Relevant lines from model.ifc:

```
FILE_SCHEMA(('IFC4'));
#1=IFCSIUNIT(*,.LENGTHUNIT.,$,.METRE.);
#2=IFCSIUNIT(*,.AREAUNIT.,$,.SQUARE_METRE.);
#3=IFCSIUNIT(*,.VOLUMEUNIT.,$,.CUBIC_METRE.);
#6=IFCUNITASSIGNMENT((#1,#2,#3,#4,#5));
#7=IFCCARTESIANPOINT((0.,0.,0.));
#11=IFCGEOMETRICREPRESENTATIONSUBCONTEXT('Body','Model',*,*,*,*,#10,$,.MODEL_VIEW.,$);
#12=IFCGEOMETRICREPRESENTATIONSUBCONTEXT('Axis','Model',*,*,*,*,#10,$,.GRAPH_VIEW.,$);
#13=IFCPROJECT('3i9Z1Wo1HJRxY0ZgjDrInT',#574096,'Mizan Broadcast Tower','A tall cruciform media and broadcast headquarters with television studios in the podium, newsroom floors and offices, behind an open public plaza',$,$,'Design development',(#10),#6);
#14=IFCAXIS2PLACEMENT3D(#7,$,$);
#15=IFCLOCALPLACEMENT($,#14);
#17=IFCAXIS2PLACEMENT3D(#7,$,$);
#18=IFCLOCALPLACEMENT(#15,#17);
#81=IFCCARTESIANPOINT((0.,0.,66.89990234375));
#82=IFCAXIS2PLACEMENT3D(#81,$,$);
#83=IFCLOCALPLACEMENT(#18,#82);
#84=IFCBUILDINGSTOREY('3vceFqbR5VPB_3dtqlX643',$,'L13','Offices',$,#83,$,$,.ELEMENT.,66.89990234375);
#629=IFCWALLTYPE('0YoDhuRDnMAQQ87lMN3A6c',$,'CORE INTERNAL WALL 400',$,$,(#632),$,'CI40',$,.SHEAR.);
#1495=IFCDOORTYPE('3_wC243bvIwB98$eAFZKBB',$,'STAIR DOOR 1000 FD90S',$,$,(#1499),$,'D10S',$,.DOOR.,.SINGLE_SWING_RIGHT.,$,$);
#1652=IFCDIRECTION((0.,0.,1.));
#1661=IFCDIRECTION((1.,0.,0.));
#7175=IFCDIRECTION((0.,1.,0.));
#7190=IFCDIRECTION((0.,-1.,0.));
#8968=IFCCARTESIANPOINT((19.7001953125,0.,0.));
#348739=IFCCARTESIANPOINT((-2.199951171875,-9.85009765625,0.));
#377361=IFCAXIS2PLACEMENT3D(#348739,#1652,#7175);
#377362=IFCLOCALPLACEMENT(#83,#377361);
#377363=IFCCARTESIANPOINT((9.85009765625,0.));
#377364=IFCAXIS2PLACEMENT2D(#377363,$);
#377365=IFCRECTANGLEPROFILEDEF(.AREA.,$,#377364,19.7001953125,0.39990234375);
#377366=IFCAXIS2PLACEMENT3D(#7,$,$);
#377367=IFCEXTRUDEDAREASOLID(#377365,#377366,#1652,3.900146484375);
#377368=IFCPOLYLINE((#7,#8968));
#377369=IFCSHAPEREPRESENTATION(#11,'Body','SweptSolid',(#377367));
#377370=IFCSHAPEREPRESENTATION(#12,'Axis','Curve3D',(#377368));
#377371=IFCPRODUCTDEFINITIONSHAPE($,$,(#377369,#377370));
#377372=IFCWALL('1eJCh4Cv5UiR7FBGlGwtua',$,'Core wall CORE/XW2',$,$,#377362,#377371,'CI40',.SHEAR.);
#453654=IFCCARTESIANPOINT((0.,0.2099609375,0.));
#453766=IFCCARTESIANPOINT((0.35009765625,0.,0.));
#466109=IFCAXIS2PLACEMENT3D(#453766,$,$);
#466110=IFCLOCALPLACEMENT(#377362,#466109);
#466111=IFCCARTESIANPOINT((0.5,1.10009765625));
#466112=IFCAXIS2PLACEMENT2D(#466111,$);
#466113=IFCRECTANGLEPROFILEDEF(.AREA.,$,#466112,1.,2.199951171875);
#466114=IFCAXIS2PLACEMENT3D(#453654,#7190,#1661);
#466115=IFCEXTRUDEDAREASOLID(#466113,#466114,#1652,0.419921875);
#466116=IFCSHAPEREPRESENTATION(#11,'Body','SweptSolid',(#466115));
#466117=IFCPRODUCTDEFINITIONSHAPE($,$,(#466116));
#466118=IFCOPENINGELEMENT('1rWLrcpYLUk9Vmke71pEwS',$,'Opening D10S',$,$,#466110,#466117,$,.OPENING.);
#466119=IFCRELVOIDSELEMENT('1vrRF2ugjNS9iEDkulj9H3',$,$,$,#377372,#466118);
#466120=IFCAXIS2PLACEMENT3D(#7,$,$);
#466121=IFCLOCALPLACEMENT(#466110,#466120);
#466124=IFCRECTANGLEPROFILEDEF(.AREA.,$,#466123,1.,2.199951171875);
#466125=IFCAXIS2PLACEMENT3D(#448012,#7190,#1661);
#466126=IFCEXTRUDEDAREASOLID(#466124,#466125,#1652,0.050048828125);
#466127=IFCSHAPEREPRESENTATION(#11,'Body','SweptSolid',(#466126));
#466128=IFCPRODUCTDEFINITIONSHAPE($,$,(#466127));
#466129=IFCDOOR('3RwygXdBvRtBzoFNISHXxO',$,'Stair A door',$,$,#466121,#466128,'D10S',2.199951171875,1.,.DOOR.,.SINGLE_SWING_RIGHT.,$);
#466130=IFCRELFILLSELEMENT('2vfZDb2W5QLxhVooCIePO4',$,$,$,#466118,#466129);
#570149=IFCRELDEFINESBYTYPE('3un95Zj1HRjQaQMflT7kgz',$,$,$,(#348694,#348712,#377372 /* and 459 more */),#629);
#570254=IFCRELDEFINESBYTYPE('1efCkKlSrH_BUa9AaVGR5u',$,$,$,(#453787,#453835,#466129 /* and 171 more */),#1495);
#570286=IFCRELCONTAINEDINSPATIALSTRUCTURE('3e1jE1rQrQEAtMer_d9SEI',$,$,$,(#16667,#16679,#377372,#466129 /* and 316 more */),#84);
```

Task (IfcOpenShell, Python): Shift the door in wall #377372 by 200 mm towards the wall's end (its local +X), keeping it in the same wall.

```python
import ifcopenshell
import ifcopenshell.api.geometry
import ifcopenshell.util.placement
import ifcopenshell.util.unit

model = ifcopenshell.open("model.ifc")
unit_scale = ifcopenshell.util.unit.calculate_unit_scale(model)

door = model.by_id(466129)
opening = door.FillsVoids[0].RelatingOpeningElement
wall = opening.VoidsElements[0].RelatingBuildingElement

wall_matrix = ifcopenshell.util.placement.get_local_placement(wall.ObjectPlacement)
shift = wall_matrix[:3, 0] * 0.2 / unit_scale
before = ifcopenshell.util.placement.get_local_placement(door.ObjectPlacement)[:3, 3].copy()

# The door is placed relative to its opening, so it follows when the opening moves.
matrix = ifcopenshell.util.placement.get_local_placement(opening.ObjectPlacement)
matrix[:3, 3] += shift
ifcopenshell.api.geometry.edit_object_placement(
    model, product=opening, matrix=matrix, is_si=False, should_transform_children=True
)

after = ifcopenshell.util.placement.get_local_placement(door.ObjectPlacement)[:3, 3]
print("door moved by", (after - before).round(3) + 0.0)

model.write("model_v2.ifc")
```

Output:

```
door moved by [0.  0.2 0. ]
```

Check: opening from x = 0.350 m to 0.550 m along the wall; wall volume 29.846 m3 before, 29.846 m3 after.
